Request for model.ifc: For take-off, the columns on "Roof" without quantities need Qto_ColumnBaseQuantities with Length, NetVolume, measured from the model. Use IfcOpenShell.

First a look at what the model holds.

```python
import ifcopenshell
import ifcopenshell.util.element
import ifcopenshell.util.unit

model = ifcopenshell.open("model.ifc")
print(model.schema)
for unit_type in ("LENGTHUNIT", "AREAUNIT", "VOLUMEUNIT"):
    print(unit_type, ifcopenshell.util.unit.calculate_unit_scale(model, unit_type))
storey = next(s for s in model.by_type("IfcBuildingStorey") if s.Name == "Roof")
columns = [e for e in ifcopenshell.util.element.get_decomposition(storey) if e.is_a("IfcColumn")]
for e in sorted(columns, key=lambda e: e.id()):
    print(e.id(), e.is_a(), e.Name, list(ifcopenshell.util.element.get_psets(e, qtos_only=True)), sep=" | ")
```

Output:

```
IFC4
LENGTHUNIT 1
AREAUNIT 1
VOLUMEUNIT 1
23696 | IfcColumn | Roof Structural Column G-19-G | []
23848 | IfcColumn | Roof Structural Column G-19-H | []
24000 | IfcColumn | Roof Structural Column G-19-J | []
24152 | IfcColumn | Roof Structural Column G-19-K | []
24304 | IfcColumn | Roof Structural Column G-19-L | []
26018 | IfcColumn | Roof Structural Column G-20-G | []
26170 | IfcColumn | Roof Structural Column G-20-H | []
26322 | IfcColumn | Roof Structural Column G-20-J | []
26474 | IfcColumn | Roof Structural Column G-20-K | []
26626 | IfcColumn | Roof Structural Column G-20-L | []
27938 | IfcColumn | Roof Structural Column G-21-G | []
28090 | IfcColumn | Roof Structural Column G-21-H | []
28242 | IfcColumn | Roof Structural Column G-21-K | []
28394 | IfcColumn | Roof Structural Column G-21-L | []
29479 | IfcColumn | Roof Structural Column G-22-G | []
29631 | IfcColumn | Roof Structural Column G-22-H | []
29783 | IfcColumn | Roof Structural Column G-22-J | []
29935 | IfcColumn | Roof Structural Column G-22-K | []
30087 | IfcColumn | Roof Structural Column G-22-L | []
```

```python
import ifcopenshell
import ifcopenshell.api.pset
import ifcopenshell.geom
import ifcopenshell.util.element
import ifcopenshell.util.shape
import ifcopenshell.util.unit

model = ifcopenshell.open("model.ifc")
unit_scale = ifcopenshell.util.unit.calculate_unit_scale(model)
volume_scale = ifcopenshell.util.unit.calculate_unit_scale(model, "VOLUMEUNIT")
settings = ifcopenshell.geom.settings()

storey = next(s for s in model.by_type("IfcBuildingStorey") if s.Name == "Roof")
columns = [e for e in ifcopenshell.util.element.get_decomposition(storey) if e.is_a("IfcColumn")]

for e in sorted(columns, key=lambda e: e.id()):
    if ifcopenshell.util.element.get_psets(e, qtos_only=True, should_inherit=False):
        continue
    # Geometry comes back in metres, in the element's own axes.
    shape = ifcopenshell.geom.create_shape(settings, e)
    values = {
        "Length": ifcopenshell.util.shape.get_z(shape.geometry) / unit_scale,
        "NetVolume": ifcopenshell.util.shape.get_volume(shape.geometry) / volume_scale,
    }
    qto = ifcopenshell.api.pset.add_qto(model, product=e, name="Qto_ColumnBaseQuantities")
    ifcopenshell.api.pset.edit_qto(model, qto=qto, properties=values)
    print(e.id(), {k: round(v, 3) for k, v in values.items()})

model.write("model_edited.ifc")
```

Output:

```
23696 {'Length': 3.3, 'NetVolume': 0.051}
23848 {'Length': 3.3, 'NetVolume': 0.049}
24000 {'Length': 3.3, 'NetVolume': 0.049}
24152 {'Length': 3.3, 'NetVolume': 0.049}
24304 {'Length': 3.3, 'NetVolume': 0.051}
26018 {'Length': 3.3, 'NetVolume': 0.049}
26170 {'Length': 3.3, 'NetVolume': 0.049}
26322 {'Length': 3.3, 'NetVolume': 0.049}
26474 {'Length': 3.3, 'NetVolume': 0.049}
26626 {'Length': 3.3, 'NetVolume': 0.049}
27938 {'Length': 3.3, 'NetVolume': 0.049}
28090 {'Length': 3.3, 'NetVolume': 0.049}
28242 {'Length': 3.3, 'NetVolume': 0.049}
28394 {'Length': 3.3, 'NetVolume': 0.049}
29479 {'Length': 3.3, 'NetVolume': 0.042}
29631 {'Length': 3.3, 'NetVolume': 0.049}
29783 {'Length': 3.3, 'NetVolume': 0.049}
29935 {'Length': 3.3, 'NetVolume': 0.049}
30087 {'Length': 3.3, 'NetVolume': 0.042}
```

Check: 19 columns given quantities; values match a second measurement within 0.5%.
